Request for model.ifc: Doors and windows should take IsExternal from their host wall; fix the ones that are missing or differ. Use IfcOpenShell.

First a look at what the model holds.

```python
import ifcopenshell
import ifcopenshell.util.element

model = ifcopenshell.open("model.ifc")
print(model.schema)
seen = {}
for e in model.by_type("IfcDoor") + model.by_type("IfcWindow"):
    if not e.FillsVoids:
        continue
    host = e.FillsVoids[0].RelatingOpeningElement.VoidsElements[0].RelatingBuildingElement
    own = ifcopenshell.util.element.get_pset(e, f"Pset_{e.is_a()[3:].removesuffix('StandardCase')}Common", "IsExternal")
    wall = ifcopenshell.util.element.get_pset(host, "Pset_WallCommon", "IsExternal")
    seen[e.is_a(), own, wall] = seen.get((e.is_a(), own, wall), 0) + 1
for (cls, own, wall), count in sorted(seen.items(), key=str):
    print(count, cls, "IsExternal:", own, "| host wall:", wall)
```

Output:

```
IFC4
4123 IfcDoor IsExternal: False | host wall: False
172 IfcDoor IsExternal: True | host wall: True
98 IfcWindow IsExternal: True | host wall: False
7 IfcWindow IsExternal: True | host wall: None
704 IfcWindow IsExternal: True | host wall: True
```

```python
import ifcopenshell
import ifcopenshell.api.pset
import ifcopenshell.util.element

model = ifcopenshell.open("model.ifc")

count = 0
for ifc_class, pset_name in (("IfcDoor", "Pset_DoorCommon"), ("IfcWindow", "Pset_WindowCommon")):
    for e in model.by_type(ifc_class):
        if not e.FillsVoids:
            continue
        host = e.FillsVoids[0].RelatingOpeningElement.VoidsElements[0].RelatingBuildingElement
        external = ifcopenshell.util.element.get_pset(host, "Pset_WallCommon", "IsExternal")
        if external is None or ifcopenshell.util.element.get_pset(e, pset_name, "IsExternal") == external:
            continue
        found = ifcopenshell.util.element.get_pset(e, pset_name, should_inherit=False)
        if found:
            pset = model.by_id(found["id"])
            if len(ifcopenshell.util.element.get_elements_by_pset(pset)) > 1:
                pset = ifcopenshell.api.pset.unshare_pset(model, products=[e], pset=pset)[0]
        else:
            pset = ifcopenshell.api.pset.add_pset(model, product=e, name=pset_name)
        ifcopenshell.api.pset.edit_pset(model, pset=pset, properties={"IsExternal": external})
        count += 1

print(count, "updated")

model.write("model_rev.ifc")
```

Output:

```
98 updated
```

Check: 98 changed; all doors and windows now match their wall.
